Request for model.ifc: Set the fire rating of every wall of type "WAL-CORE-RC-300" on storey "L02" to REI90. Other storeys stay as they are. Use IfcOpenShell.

First a look at what the model holds.

```python
import ifcopenshell
import ifcopenshell.util.element

model = ifcopenshell.open("model.ifc")
print(model.schema)
storey = next(s for s in model.by_type("IfcBuildingStorey") if s.Name == "L02")
walls = [e for e in ifcopenshell.util.element.get_decomposition(storey) if e.is_a("IfcWall")]
seen = {}
for e in walls:
    element_type = ifcopenshell.util.element.get_type(e)
    key = (element_type.Name if element_type != e and element_type else None, ifcopenshell.util.element.get_pset(e, "Pset_WallCommon", "FireRating"))
    seen[key] = seen.get(key, 0) + 1
for (name, value), count in sorted(seen.items(), key=str):
    print(count, "x", name, "|", value)
```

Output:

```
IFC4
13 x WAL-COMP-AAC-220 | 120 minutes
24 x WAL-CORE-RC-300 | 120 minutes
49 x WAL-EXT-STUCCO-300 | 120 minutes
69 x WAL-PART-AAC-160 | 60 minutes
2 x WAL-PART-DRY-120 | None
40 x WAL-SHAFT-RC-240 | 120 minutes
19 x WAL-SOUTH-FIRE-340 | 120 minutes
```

```python
import ifcopenshell
import ifcopenshell.api.pset
import ifcopenshell.util.element

model = ifcopenshell.open("model.ifc")

storey = next(s for s in model.by_type("IfcBuildingStorey") if s.Name == "L02")
walls = [e for e in ifcopenshell.util.element.get_decomposition(storey) if e.is_a("IfcWall")]

count = 0
for e in walls:
    element_type = ifcopenshell.util.element.get_type(e)
    if element_type in (None, e) or element_type.Name != "WAL-CORE-RC-300":
        continue
    # add_pset returns the element's existing set when there is one.
    pset = ifcopenshell.api.pset.add_pset(model, product=e, name="Pset_WallCommon")
    ifcopenshell.api.pset.edit_pset(model, pset=pset, properties={"FireRating": "REI90"})
    count += 1

print(count, "walls updated")

model.write("model_edited.ifc")
```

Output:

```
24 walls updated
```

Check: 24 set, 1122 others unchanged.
